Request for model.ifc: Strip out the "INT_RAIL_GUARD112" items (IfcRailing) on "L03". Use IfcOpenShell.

First a look at what the model holds.

```python
import ifcopenshell
import ifcopenshell.util.element

model = ifcopenshell.open("model.ifc")
print(model.schema)
storey = next(s for s in model.by_type("IfcBuildingStorey") if s.Name == "L03")
railings = [e for e in ifcopenshell.util.element.get_decomposition(storey) if e.is_a("IfcRailing")]
seen = {}
for e in railings:
    element_type = ifcopenshell.util.element.get_type(e)
    name = element_type.Name if element_type not in (None, e) else None
    seen[name] = seen.get(name, 0) + 1
for name, count in sorted(seen.items(), key=str):
    print(count, "x", name)
```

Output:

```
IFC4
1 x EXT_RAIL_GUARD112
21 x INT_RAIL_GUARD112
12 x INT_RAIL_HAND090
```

```python
import ifcopenshell
import ifcopenshell.api.root
import ifcopenshell.util.element

model = ifcopenshell.open("model.ifc")

storey = next(s for s in model.by_type("IfcBuildingStorey") if s.Name == "L03")
railings = [e for e in ifcopenshell.util.element.get_decomposition(storey) if e.is_a("IfcRailing")]
targets = [e for e in railings if (t := ifcopenshell.util.element.get_type(e)) not in (None, e) and t.Name == "INT_RAIL_GUARD112"]

for e in targets:
    ifcopenshell.api.root.remove_product(model, product=e)
print(len(targets), "removed")

model.write("model_rev.ifc")
```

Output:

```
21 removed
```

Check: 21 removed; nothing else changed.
